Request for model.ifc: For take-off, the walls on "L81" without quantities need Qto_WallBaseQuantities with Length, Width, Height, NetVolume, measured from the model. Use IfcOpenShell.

First a look at what the model holds.

```python
import ifcopenshell
import ifcopenshell.util.element
import ifcopenshell.util.unit

model = ifcopenshell.open("model.ifc")
print(model.schema)
for unit_type in ("LENGTHUNIT", "AREAUNIT", "VOLUMEUNIT"):
    print(unit_type, ifcopenshell.util.unit.calculate_unit_scale(model, unit_type))
storey = next(s for s in model.by_type("IfcBuildingStorey") if s.Name == "L81")
walls = [e for e in ifcopenshell.util.element.get_decomposition(storey) if e.is_a("IfcWall")]
for e in sorted(walls, key=lambda e: e.id()):
    print(e.id(), e.is_a(), e.Name, list(ifcopenshell.util.element.get_psets(e, qtos_only=True)), sep=" | ")
```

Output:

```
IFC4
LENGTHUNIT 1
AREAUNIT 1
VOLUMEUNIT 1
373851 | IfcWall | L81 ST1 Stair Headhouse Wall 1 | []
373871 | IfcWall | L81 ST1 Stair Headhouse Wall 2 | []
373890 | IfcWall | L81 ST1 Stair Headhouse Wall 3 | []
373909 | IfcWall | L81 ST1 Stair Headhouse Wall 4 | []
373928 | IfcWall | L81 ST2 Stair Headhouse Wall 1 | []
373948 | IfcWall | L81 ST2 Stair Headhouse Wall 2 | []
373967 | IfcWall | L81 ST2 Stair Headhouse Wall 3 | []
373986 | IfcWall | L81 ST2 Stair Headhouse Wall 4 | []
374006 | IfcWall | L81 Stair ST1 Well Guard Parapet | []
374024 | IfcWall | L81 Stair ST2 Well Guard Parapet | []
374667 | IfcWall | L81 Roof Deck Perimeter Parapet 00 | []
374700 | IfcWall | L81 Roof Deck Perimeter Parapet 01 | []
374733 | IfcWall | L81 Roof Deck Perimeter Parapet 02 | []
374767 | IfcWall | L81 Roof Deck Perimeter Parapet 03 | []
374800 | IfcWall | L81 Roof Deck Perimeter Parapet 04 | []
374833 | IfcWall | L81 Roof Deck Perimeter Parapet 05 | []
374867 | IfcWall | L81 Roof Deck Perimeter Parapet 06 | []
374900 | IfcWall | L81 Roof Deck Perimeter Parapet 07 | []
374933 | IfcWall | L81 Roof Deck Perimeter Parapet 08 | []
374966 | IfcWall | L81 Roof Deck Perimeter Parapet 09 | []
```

```python
import ifcopenshell
import ifcopenshell.api.pset
import ifcopenshell.geom
import ifcopenshell.util.element
import ifcopenshell.util.shape
import ifcopenshell.util.unit

model = ifcopenshell.open("model.ifc")
unit_scale = ifcopenshell.util.unit.calculate_unit_scale(model)
volume_scale = ifcopenshell.util.unit.calculate_unit_scale(model, "VOLUMEUNIT")
settings = ifcopenshell.geom.settings()

storey = next(s for s in model.by_type("IfcBuildingStorey") if s.Name == "L81")
walls = [e for e in ifcopenshell.util.element.get_decomposition(storey) if e.is_a("IfcWall")]

for e in sorted(walls, key=lambda e: e.id()):
    if ifcopenshell.util.element.get_psets(e, qtos_only=True, should_inherit=False):
        continue
    # Geometry comes back in metres, in the element's own axes.
    shape = ifcopenshell.geom.create_shape(settings, e)
    values = {
        "Length": ifcopenshell.util.shape.get_x(shape.geometry) / unit_scale,
        "Width": ifcopenshell.util.shape.get_y(shape.geometry) / unit_scale,
        "Height": ifcopenshell.util.shape.get_z(shape.geometry) / unit_scale,
        "NetVolume": ifcopenshell.util.shape.get_volume(shape.geometry) / volume_scale,
    }
    qto = ifcopenshell.api.pset.add_qto(model, product=e, name="Qto_WallBaseQuantities")
    ifcopenshell.api.pset.edit_qto(model, qto=qto, properties=values)
    print(e.id(), {k: round(v, 3) for k, v in values.items()})

model.write("model_updated.ifc")
```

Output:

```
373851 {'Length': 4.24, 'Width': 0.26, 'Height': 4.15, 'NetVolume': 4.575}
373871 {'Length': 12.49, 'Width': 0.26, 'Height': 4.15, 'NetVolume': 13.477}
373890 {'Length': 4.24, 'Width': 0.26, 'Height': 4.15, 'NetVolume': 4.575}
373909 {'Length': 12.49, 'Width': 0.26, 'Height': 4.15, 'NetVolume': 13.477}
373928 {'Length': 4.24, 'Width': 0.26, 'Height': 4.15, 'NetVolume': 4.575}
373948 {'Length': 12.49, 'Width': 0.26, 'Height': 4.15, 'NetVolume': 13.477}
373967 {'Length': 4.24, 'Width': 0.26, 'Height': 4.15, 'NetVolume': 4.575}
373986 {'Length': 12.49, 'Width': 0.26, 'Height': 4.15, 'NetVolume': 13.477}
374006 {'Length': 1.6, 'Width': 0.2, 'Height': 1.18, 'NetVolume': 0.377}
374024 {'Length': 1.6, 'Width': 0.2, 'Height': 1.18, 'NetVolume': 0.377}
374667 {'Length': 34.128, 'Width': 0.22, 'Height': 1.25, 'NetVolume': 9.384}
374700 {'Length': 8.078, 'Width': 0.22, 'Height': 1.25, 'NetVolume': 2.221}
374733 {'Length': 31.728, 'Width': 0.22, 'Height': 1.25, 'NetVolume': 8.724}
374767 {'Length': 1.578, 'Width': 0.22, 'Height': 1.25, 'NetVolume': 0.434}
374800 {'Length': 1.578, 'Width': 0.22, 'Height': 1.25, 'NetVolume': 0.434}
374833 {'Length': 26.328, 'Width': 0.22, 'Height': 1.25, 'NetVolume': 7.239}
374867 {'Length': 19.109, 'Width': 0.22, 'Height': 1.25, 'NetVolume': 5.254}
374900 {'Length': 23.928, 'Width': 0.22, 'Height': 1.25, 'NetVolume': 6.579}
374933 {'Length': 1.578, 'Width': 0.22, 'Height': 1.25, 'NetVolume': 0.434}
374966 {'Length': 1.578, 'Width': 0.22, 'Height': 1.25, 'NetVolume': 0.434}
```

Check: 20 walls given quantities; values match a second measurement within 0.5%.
